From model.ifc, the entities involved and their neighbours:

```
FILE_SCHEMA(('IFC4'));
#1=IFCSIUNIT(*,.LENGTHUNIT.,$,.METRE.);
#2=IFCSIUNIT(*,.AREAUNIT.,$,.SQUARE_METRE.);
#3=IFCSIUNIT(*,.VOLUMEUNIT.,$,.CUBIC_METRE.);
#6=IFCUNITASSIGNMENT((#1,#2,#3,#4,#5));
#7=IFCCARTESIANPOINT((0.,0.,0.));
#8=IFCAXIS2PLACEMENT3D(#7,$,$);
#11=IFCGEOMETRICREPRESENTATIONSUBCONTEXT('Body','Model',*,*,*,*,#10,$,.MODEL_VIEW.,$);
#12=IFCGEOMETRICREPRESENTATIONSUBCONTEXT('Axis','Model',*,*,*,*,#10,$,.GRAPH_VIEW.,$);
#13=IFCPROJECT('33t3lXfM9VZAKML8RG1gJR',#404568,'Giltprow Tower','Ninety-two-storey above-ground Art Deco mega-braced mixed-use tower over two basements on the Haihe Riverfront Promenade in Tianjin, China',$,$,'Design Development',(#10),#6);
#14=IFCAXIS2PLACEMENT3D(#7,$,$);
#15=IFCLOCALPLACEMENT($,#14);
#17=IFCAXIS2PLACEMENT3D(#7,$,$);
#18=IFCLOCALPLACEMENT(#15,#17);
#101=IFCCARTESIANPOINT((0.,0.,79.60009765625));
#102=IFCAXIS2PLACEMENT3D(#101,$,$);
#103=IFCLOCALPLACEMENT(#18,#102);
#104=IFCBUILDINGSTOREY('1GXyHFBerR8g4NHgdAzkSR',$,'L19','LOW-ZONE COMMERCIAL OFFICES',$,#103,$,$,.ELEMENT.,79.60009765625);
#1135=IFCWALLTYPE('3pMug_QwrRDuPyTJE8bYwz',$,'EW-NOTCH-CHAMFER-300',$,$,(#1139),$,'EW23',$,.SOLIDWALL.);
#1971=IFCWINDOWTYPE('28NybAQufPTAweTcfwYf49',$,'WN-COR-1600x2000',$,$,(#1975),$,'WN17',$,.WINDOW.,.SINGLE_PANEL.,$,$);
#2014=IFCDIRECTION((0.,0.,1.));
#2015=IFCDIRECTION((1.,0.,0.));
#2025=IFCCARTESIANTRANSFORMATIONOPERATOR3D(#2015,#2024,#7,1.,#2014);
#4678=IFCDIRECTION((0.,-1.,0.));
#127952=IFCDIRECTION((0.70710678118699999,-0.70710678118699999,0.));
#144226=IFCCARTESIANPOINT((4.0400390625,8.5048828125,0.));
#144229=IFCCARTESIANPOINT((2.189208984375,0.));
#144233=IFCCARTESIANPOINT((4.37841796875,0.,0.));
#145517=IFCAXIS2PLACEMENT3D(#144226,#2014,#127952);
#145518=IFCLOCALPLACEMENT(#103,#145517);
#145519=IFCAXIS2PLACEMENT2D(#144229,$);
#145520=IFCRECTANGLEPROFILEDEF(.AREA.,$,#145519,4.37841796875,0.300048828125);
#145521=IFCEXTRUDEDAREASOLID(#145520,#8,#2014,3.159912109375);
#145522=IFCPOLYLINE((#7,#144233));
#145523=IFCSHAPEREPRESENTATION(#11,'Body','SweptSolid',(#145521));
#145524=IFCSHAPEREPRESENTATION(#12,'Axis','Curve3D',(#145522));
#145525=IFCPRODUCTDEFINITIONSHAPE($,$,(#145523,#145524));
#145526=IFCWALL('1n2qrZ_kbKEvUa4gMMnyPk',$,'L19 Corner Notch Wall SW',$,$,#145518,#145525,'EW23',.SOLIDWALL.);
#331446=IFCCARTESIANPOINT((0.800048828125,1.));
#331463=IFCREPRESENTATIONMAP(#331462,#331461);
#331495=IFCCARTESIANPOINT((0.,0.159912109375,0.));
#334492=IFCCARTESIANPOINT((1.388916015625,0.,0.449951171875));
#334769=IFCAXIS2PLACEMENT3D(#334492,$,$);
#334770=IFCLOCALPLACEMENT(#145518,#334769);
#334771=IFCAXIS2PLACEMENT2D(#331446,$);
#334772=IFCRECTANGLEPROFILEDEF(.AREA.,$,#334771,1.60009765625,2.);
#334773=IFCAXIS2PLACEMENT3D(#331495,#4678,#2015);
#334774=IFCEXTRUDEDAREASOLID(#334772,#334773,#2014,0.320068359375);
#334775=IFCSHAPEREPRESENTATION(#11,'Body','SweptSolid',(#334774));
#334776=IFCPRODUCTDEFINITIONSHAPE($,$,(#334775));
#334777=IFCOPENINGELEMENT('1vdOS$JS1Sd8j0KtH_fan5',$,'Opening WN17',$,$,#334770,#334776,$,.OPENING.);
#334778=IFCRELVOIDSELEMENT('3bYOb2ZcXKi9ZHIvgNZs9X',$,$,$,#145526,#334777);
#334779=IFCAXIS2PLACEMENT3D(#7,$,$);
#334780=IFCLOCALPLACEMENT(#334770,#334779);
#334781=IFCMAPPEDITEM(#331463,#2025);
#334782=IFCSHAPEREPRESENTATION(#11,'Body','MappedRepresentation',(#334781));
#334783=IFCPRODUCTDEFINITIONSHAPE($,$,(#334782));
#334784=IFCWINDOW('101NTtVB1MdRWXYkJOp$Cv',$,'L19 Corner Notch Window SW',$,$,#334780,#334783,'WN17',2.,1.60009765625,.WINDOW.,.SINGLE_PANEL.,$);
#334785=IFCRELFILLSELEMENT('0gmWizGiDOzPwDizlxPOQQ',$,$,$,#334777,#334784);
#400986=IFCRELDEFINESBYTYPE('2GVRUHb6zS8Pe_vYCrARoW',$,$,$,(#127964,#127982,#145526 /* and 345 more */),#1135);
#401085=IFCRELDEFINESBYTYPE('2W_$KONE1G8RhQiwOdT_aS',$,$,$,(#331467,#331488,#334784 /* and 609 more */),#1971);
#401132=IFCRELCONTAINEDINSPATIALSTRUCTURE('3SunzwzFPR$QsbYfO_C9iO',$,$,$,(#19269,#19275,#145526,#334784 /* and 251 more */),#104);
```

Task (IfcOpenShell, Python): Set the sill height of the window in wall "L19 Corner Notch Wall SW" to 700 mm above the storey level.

```python
import numpy as np
import ifcopenshell
import ifcopenshell.api.geometry
import ifcopenshell.geom
import ifcopenshell.util.element
import ifcopenshell.util.placement
import ifcopenshell.util.shape
import ifcopenshell.util.unit

model = ifcopenshell.open("model.ifc")
unit_scale = ifcopenshell.util.unit.calculate_unit_scale(model)

window = model.by_id(334784)
opening = window.FillsVoids[0].RelatingOpeningElement
storey = ifcopenshell.util.element.get_container(window, ifc_class="IfcBuildingStorey")
level = ifcopenshell.util.placement.get_local_placement(storey.ObjectPlacement)[2, 3]

# The opening's origin need not be at the sill, so measure its lowest point.
shape = ifcopenshell.geom.create_shape(ifcopenshell.geom.settings(), opening)
bottom = ifcopenshell.util.shape.get_shape_bottom_elevation(shape, shape.geometry) / unit_scale
dz = level + 0.7 / unit_scale - bottom

shift = np.array([0.0, 0.0, dz])
# The window is placed relative to its opening, so it follows when the opening moves.
matrix = ifcopenshell.util.placement.get_local_placement(opening.ObjectPlacement)
matrix[:3, 3] += shift
ifcopenshell.api.geometry.edit_object_placement(
    model, product=opening, matrix=matrix, is_si=False, should_transform_children=True
)

print(f"moved by {dz * unit_scale:+.3f} m")

model.write("model_rev.ifc")
```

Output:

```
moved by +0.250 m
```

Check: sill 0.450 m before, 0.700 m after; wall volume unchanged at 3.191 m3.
